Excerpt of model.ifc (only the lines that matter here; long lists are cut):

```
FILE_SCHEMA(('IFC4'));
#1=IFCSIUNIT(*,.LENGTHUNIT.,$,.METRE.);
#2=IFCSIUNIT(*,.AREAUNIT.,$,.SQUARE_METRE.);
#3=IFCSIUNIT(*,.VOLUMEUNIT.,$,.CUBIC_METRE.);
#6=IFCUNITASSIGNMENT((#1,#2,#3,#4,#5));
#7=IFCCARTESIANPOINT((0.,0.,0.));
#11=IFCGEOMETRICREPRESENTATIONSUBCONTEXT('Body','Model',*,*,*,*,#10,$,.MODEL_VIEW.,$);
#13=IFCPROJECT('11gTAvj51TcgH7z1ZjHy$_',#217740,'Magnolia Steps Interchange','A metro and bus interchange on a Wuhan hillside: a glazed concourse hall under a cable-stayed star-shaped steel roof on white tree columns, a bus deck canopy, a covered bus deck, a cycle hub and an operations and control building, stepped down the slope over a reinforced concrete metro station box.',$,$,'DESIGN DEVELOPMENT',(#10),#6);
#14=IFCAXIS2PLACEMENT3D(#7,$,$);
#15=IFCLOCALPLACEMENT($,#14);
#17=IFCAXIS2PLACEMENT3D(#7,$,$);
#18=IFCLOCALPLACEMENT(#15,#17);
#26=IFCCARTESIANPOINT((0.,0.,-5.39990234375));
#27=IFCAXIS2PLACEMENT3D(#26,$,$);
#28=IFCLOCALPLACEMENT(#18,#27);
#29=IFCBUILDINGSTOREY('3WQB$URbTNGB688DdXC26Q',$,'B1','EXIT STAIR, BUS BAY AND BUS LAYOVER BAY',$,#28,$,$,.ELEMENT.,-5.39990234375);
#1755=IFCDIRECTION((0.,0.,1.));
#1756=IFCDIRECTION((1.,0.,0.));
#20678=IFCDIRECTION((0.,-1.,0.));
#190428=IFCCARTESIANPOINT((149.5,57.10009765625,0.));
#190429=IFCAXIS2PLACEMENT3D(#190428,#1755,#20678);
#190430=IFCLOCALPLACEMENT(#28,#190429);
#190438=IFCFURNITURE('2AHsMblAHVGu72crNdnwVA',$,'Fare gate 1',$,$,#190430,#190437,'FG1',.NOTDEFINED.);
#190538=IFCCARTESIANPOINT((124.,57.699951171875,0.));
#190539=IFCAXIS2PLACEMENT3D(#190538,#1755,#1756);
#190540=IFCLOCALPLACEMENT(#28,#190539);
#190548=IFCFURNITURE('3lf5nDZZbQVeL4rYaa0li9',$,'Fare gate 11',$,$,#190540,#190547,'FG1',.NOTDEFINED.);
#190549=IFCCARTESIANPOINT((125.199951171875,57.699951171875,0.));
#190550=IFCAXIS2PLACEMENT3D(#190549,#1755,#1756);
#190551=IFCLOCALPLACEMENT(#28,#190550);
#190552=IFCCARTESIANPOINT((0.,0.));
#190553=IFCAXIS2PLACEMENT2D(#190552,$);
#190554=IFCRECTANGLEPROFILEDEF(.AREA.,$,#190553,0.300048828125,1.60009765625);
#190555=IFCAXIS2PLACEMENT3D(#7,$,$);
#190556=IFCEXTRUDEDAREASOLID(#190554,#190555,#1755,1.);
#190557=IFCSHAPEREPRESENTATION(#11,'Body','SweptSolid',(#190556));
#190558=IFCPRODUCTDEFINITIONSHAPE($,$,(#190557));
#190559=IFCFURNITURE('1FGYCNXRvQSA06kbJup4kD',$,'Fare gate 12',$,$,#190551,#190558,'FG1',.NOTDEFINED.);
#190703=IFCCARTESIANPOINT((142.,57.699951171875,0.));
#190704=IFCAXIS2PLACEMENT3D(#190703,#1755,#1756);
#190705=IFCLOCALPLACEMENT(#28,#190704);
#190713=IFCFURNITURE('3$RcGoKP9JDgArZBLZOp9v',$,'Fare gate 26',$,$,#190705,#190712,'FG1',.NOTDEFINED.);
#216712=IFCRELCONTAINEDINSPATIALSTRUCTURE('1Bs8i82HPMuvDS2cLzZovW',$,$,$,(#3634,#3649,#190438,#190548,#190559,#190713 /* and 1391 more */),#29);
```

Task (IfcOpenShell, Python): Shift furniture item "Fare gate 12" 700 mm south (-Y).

```python
import ifcopenshell
import ifcopenshell.api.geometry
import ifcopenshell.util.placement

model = ifcopenshell.open("model.ifc")

item = model.by_id(190559)
matrix = ifcopenshell.util.placement.get_local_placement(item.ObjectPlacement)
matrix[1, 3] -= 0.7
ifcopenshell.api.geometry.edit_object_placement(model, product=item, matrix=matrix, is_si=False)

print(ifcopenshell.util.placement.get_local_placement(item.ObjectPlacement).round(3) + 0.0)

model.write("model_updated.ifc")
```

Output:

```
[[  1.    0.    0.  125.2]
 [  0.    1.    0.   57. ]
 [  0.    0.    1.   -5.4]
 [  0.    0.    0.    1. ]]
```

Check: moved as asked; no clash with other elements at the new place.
